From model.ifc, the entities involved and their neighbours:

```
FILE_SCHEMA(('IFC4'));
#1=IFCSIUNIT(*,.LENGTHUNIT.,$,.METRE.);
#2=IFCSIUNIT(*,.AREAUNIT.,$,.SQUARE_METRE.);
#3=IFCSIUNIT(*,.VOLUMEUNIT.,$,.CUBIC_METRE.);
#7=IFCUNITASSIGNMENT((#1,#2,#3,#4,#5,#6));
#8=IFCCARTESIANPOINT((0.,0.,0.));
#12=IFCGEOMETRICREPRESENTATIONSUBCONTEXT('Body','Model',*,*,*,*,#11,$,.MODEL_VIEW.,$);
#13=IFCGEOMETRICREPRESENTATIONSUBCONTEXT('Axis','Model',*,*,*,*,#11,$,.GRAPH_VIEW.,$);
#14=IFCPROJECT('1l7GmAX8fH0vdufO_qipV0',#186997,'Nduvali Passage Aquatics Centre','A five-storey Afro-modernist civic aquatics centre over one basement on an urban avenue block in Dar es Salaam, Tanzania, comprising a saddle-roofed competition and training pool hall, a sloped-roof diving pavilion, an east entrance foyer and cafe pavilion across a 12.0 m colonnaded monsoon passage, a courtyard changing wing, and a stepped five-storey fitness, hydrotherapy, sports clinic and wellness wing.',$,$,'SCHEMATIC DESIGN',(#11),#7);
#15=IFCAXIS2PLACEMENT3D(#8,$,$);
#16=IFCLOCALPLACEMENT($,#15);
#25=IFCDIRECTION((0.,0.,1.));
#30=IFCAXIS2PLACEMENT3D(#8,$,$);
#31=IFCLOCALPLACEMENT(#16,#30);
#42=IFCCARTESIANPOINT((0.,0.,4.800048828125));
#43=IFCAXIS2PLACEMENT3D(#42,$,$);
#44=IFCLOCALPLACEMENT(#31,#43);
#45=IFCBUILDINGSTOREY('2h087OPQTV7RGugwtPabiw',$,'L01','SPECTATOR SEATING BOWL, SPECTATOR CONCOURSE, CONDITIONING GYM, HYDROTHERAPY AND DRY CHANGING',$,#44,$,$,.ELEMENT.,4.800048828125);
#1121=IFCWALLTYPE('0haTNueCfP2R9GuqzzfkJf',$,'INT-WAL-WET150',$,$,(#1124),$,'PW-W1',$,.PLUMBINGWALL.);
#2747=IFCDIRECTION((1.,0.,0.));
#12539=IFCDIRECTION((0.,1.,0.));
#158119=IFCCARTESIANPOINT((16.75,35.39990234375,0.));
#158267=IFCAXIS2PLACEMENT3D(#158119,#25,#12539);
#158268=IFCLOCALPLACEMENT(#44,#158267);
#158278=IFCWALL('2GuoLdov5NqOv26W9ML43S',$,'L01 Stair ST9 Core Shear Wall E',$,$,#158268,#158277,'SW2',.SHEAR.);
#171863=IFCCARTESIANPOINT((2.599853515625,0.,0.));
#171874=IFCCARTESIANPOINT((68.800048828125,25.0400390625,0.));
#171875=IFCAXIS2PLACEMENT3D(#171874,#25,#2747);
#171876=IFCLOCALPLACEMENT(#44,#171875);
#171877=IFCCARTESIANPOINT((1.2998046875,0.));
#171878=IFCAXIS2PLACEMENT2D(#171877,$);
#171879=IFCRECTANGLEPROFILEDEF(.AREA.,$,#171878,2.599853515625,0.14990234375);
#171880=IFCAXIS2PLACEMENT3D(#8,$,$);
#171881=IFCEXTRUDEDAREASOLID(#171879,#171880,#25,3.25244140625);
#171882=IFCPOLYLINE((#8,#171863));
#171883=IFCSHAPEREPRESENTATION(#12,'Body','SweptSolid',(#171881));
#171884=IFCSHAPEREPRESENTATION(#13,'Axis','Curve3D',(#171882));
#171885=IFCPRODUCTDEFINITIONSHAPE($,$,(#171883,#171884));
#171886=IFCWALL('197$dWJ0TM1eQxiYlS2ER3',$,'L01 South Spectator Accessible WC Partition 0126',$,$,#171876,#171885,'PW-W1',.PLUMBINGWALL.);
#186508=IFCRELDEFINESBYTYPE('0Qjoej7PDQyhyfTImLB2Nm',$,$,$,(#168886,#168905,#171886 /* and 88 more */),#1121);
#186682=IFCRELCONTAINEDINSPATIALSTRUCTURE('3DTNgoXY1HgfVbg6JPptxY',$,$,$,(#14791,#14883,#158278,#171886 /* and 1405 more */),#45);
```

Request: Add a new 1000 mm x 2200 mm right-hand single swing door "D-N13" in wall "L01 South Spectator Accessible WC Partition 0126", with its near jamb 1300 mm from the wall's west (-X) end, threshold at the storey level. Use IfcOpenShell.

```python
import numpy as np
import ifcopenshell
import ifcopenshell.api.feature
import ifcopenshell.api.geometry
import ifcopenshell.api.root
import ifcopenshell.api.spatial
import ifcopenshell.geom
import ifcopenshell.util.element
import ifcopenshell.util.placement
import ifcopenshell.util.representation
import ifcopenshell.util.shape
import ifcopenshell.util.unit

model = ifcopenshell.open("model.ifc")
unit_scale = ifcopenshell.util.unit.calculate_unit_scale(model)
settings = ifcopenshell.geom.settings()


def volume(element):
    """Net volume in cubic metres, openings subtracted."""
    shape = ifcopenshell.geom.create_shape(settings, element)
    return ifcopenshell.util.shape.get_volume(shape.geometry)


wall = model.by_guid("197$dWJ0TM1eQxiYlS2ER3")
storey = ifcopenshell.util.element.get_container(wall, ifc_class="IfcBuildingStorey")
context = ifcopenshell.util.representation.get_context(model, "Model", "Body", "MODEL_VIEW")
before = volume(wall)

width, height, from_end, sill = 1, 2.2, 1.3, 0.0  # metres

# The wall runs along its own X axis, and the end named is its -X end.
wall_shape = ifcopenshell.geom.create_shape(settings, wall)
x, y, z = ifcopenshell.util.shape.get_vertices(wall_shape.geometry).T
start = x.min() + from_end
face, thickness = float(y.min()), float(y.max() - y.min())
wall_matrix = ifcopenshell.util.placement.get_local_placement(wall.ObjectPlacement)
level = ifcopenshell.util.placement.get_local_placement(storey.ObjectPlacement)[2, 3]


def in_wall(x, y):
    """Placement at x, y metres in the wall's axes, at sill height."""
    matrix = wall_matrix.copy()
    matrix[:, 3] = wall_matrix @ np.array([x / unit_scale, y / unit_scale, 0.0, 1.0])
    matrix[2, 3] = level + sill / unit_scale
    return matrix


# Opening: a box that overshoots both wall faces by 50 mm.
opening = ifcopenshell.api.root.create_entity(model, ifc_class="IfcOpeningElement", predefined_type="OPENING")
box = ifcopenshell.api.geometry.add_wall_representation(
    model, context=context, length=width, height=height, thickness=thickness + 0.1
)
ifcopenshell.api.geometry.assign_representation(model, product=opening, representation=box)
ifcopenshell.api.geometry.edit_object_placement(model, product=opening, matrix=in_wall(start, face - 0.05), is_si=False)
ifcopenshell.api.feature.add_feature(model, feature=opening, element=wall)

door = ifcopenshell.api.root.create_entity(model, ifc_class="IfcDoor", name="D-N13", predefined_type="DOOR")
door.OverallWidth, door.OverallHeight = width / unit_scale, height / unit_scale
door.OperationType = "SINGLE_SWING_RIGHT"
body = ifcopenshell.api.geometry.add_door_representation(
    model,
    context=context,
    overall_width=door.OverallWidth,
    overall_height=door.OverallHeight,
    operation_type="SINGLE_SWING_RIGHT",
    lining_properties={"LiningDepth": thickness / unit_scale, "ThresholdDepth": thickness / unit_scale},
)
ifcopenshell.api.geometry.assign_representation(model, product=door, representation=body)
ifcopenshell.api.spatial.assign_container(model, products=[door], relating_structure=storey)
ifcopenshell.api.feature.add_filling(model, opening=opening, element=door)

# The lining spans the wall, so the door starts at the wall face.
ifcopenshell.api.geometry.edit_object_placement(model, product=door, matrix=in_wall(start, face), is_si=False)

after = volume(wall)

print(f"wall volume {before:.3f} -> {after:.3f} m3")

model.write("model_rev.ifc")
```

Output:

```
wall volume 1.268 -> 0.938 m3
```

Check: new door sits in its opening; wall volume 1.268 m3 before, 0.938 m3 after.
